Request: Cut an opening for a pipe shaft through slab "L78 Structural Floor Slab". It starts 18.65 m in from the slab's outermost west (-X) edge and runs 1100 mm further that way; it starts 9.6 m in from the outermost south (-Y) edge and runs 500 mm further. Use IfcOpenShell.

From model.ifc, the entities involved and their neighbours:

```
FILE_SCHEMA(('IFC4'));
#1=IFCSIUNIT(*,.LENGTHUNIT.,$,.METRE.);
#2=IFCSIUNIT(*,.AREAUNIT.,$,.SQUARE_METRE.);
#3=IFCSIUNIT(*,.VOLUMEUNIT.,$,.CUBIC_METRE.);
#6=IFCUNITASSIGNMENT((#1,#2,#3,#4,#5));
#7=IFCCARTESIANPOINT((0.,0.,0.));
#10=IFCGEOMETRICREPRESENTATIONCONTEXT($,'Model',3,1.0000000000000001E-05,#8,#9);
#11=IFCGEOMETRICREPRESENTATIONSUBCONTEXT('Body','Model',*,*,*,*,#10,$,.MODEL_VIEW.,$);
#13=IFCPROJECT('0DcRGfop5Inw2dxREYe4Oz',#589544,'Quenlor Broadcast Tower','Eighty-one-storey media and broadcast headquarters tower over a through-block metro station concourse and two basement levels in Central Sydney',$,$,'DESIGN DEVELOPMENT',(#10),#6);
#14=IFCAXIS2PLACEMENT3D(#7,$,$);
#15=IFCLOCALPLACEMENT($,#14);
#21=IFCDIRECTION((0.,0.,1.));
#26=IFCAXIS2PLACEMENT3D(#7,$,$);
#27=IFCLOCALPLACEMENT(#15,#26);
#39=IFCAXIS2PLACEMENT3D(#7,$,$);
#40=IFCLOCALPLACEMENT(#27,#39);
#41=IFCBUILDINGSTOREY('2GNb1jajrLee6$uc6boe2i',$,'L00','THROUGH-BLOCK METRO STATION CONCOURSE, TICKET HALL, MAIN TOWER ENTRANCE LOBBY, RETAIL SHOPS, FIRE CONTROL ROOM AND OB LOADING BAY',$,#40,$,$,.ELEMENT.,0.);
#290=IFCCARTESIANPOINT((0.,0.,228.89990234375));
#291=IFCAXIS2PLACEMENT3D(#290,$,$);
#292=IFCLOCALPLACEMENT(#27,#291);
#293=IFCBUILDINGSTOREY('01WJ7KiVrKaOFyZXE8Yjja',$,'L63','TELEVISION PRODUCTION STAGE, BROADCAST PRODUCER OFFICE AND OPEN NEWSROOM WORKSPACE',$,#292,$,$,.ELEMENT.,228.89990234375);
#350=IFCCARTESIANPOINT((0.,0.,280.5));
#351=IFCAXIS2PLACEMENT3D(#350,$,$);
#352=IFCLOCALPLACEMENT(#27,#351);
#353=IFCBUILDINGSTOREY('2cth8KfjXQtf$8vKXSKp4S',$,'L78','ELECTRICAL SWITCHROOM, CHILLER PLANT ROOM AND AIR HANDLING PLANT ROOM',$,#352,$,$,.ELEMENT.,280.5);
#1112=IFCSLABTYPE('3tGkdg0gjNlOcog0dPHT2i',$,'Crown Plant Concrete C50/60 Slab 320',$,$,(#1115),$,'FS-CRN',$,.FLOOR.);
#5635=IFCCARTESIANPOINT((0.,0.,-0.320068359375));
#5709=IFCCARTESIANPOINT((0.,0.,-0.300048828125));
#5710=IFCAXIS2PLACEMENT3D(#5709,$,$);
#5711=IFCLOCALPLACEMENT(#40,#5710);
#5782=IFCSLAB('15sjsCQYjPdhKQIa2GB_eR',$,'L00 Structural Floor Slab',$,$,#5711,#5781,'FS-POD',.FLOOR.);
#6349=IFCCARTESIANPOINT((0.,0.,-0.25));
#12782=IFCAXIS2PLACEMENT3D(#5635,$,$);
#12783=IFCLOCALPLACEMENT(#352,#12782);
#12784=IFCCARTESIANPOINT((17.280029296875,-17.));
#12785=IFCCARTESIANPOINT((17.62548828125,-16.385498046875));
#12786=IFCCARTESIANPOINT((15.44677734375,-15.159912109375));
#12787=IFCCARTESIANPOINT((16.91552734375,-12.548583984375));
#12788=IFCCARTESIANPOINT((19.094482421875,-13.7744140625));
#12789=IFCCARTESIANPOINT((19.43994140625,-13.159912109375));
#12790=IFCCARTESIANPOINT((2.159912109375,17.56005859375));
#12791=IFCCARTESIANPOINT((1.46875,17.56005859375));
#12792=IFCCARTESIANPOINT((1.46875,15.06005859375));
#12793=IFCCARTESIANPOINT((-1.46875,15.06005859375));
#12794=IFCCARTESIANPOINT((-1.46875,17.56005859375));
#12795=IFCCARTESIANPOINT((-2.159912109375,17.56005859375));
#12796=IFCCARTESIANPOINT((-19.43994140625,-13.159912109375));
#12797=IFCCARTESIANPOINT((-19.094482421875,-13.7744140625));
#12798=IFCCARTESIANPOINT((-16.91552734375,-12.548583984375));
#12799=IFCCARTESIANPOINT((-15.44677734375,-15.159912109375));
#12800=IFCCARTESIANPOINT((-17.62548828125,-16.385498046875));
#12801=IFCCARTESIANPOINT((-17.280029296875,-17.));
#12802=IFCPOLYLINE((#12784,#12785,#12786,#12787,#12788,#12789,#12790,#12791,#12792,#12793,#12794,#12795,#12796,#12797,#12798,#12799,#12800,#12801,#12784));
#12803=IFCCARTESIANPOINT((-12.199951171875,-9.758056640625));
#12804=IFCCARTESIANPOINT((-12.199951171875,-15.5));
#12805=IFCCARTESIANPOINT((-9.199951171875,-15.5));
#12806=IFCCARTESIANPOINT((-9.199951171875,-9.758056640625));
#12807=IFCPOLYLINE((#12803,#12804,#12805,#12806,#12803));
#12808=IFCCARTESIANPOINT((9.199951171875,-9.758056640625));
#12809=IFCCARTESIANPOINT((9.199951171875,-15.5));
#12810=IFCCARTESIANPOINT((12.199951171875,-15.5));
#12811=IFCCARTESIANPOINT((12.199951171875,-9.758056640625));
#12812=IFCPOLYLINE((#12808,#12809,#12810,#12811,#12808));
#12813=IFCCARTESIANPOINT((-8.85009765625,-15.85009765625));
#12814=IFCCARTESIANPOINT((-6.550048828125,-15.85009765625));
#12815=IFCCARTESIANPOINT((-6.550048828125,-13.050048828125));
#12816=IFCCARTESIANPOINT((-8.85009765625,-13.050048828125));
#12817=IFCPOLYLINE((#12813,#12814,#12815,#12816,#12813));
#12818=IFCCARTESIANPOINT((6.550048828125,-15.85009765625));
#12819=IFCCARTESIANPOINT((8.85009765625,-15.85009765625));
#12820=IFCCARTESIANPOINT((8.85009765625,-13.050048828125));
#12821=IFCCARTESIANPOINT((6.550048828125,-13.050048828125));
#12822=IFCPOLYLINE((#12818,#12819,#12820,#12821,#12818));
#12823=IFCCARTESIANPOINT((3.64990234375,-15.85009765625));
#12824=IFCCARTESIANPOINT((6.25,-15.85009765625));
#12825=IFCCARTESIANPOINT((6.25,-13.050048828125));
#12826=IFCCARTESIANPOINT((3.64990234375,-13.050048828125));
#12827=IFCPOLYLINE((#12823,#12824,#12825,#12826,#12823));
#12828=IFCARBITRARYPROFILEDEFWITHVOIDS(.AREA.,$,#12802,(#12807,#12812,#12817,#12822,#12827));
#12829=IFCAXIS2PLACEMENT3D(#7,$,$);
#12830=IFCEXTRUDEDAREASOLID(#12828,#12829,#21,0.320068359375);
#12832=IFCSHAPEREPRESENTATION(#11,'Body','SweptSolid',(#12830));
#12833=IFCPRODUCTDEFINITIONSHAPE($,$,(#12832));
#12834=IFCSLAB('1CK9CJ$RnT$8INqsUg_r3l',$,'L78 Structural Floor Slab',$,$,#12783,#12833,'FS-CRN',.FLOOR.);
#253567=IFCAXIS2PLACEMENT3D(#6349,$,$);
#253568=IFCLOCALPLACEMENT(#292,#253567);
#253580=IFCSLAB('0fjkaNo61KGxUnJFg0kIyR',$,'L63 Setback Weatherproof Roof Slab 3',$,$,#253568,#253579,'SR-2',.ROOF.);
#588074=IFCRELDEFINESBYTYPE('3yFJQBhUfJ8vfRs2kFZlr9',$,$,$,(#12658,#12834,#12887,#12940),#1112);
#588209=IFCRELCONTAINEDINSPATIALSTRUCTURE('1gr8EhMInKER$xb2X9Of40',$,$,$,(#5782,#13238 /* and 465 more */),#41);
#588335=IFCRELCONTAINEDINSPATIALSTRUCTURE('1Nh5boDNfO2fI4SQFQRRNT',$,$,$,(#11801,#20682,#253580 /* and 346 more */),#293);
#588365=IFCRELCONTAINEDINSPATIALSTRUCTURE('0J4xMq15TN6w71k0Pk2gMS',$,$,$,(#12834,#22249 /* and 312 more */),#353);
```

```python
import numpy as np
import ifcopenshell
import ifcopenshell.api.feature
import ifcopenshell.api.geometry
import ifcopenshell.api.root
import ifcopenshell.geom
import ifcopenshell.util.placement
import ifcopenshell.util.representation
import ifcopenshell.util.shape
import ifcopenshell.util.unit

model = ifcopenshell.open("model.ifc")
unit_scale = ifcopenshell.util.unit.calculate_unit_scale(model)
settings = ifcopenshell.geom.settings()


def volume(element):
    """Net volume in cubic metres, openings subtracted."""
    shape = ifcopenshell.geom.create_shape(settings, element)
    return ifcopenshell.util.shape.get_volume(shape.geometry)


slab = model.by_guid("1CK9CJ$RnT$8INqsUg_r3l")
before = volume(slab)

# Extent in the slab's own axes, in metres. The edges named are its -X and -Y sides.
slab_shape = ifcopenshell.geom.create_shape(settings, slab)
vertices = ifcopenshell.util.shape.get_vertices(slab_shape.geometry)
x_min, y_min, bottom = vertices.min(axis=0)
top = vertices[:, 2].max()

opening = ifcopenshell.api.root.create_entity(model, ifc_class="IfcOpeningElement", name="Pipe shaft opening", predefined_type="OPENING")
context = ifcopenshell.util.representation.get_context(model, "Model", "Body", "MODEL_VIEW")
width, depth = 1.1, 0.5
outline = [(0.0, 0.0), (width, 0.0), (width, depth), (0.0, depth), (0.0, 0.0)]
# Overshoot both faces by 50 mm so the cut is clean.
shape = ifcopenshell.api.geometry.add_slab_representation(
    model, context=context, depth=top - bottom + 0.1, polyline=outline
)
ifcopenshell.api.geometry.assign_representation(model, product=opening, representation=shape)

matrix = ifcopenshell.util.placement.get_local_placement(slab.ObjectPlacement)
matrix[:, 3] = matrix @ np.append(np.array([x_min + 18.65, y_min + 9.6, bottom - 0.05]) / unit_scale, 1.0)
ifcopenshell.api.geometry.edit_object_placement(model, product=opening, matrix=matrix, is_si=False)
ifcopenshell.api.feature.add_feature(model, feature=opening, element=slab)

after = volume(slab)

print(f"slab volume {before:.3f} -> {after:.3f} m3")

model.write("model-out.ifc")
```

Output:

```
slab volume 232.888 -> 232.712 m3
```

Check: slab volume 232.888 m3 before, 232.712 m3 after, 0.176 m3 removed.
